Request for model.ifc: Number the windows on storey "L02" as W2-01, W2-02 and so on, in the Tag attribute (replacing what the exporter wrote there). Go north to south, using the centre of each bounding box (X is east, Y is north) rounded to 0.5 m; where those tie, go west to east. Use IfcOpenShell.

First a look at what the model holds.

```python
import ifcopenshell
import ifcopenshell.util.element
import ifcopenshell.util.placement

model = ifcopenshell.open("model.ifc")
print(model.schema)
storey = next(s for s in model.by_type("IfcBuildingStorey") if s.Name == "L02")
windows = [e for e in ifcopenshell.util.element.get_decomposition(storey) if e.is_a("IfcWindow")]
for e in sorted(windows, key=lambda e: e.id()):
    origin = ifcopenshell.util.placement.get_local_placement(e.ObjectPlacement)[:3, 3]
    print(e.id(), e.Tag, e.Name, origin.round(2) + 0.0, sep=" | ")
```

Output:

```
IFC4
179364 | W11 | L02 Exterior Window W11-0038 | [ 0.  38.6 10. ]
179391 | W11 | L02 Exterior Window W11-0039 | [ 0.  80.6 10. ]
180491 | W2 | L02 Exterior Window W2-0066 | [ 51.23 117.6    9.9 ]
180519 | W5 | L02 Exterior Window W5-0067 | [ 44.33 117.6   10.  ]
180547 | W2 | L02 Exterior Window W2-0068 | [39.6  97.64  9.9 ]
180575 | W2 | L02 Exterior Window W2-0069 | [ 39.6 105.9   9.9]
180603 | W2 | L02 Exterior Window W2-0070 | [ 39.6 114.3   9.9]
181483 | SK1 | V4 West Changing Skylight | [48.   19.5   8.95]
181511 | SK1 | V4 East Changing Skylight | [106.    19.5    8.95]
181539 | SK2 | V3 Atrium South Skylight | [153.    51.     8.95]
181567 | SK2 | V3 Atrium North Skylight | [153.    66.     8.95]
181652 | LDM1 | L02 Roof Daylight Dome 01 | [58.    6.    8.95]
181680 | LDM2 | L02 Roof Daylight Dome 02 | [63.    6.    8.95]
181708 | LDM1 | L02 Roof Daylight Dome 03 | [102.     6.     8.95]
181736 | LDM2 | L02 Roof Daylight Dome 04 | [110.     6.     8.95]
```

```python
import ifcopenshell
import ifcopenshell.geom
import ifcopenshell.util.element
import ifcopenshell.util.shape

model = ifcopenshell.open("model.ifc")
settings = ifcopenshell.geom.settings()
settings.set("use-world-coords", True)


def centre(element):
    shape = ifcopenshell.geom.create_shape(settings, element)
    return ifcopenshell.util.shape.get_bbox_centroid(shape.geometry)


storey = next(s for s in model.by_type("IfcBuildingStorey") if s.Name == "L02")
windows = [e for e in ifcopenshell.util.element.get_decomposition(storey) if e.is_a("IfcWindow")]

# Insertion points can sit at a corner or the storey origin, so sort by the geometry (in metres).
centres = {e: centre(e) for e in windows}
windows.sort(key=lambda e: (-round(centres[e][1] / 0.5), centres[e][0]))

for i, e in enumerate(windows, start=1):
    number = f"W2-{i:02d}"
    e.Tag = number
    print(e.id(), number)

model.write("model_updated.ifc")
```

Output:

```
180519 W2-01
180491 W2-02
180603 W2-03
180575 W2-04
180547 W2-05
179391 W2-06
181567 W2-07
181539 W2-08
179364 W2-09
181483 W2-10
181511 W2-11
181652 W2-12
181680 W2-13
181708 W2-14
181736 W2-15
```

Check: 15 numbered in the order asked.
